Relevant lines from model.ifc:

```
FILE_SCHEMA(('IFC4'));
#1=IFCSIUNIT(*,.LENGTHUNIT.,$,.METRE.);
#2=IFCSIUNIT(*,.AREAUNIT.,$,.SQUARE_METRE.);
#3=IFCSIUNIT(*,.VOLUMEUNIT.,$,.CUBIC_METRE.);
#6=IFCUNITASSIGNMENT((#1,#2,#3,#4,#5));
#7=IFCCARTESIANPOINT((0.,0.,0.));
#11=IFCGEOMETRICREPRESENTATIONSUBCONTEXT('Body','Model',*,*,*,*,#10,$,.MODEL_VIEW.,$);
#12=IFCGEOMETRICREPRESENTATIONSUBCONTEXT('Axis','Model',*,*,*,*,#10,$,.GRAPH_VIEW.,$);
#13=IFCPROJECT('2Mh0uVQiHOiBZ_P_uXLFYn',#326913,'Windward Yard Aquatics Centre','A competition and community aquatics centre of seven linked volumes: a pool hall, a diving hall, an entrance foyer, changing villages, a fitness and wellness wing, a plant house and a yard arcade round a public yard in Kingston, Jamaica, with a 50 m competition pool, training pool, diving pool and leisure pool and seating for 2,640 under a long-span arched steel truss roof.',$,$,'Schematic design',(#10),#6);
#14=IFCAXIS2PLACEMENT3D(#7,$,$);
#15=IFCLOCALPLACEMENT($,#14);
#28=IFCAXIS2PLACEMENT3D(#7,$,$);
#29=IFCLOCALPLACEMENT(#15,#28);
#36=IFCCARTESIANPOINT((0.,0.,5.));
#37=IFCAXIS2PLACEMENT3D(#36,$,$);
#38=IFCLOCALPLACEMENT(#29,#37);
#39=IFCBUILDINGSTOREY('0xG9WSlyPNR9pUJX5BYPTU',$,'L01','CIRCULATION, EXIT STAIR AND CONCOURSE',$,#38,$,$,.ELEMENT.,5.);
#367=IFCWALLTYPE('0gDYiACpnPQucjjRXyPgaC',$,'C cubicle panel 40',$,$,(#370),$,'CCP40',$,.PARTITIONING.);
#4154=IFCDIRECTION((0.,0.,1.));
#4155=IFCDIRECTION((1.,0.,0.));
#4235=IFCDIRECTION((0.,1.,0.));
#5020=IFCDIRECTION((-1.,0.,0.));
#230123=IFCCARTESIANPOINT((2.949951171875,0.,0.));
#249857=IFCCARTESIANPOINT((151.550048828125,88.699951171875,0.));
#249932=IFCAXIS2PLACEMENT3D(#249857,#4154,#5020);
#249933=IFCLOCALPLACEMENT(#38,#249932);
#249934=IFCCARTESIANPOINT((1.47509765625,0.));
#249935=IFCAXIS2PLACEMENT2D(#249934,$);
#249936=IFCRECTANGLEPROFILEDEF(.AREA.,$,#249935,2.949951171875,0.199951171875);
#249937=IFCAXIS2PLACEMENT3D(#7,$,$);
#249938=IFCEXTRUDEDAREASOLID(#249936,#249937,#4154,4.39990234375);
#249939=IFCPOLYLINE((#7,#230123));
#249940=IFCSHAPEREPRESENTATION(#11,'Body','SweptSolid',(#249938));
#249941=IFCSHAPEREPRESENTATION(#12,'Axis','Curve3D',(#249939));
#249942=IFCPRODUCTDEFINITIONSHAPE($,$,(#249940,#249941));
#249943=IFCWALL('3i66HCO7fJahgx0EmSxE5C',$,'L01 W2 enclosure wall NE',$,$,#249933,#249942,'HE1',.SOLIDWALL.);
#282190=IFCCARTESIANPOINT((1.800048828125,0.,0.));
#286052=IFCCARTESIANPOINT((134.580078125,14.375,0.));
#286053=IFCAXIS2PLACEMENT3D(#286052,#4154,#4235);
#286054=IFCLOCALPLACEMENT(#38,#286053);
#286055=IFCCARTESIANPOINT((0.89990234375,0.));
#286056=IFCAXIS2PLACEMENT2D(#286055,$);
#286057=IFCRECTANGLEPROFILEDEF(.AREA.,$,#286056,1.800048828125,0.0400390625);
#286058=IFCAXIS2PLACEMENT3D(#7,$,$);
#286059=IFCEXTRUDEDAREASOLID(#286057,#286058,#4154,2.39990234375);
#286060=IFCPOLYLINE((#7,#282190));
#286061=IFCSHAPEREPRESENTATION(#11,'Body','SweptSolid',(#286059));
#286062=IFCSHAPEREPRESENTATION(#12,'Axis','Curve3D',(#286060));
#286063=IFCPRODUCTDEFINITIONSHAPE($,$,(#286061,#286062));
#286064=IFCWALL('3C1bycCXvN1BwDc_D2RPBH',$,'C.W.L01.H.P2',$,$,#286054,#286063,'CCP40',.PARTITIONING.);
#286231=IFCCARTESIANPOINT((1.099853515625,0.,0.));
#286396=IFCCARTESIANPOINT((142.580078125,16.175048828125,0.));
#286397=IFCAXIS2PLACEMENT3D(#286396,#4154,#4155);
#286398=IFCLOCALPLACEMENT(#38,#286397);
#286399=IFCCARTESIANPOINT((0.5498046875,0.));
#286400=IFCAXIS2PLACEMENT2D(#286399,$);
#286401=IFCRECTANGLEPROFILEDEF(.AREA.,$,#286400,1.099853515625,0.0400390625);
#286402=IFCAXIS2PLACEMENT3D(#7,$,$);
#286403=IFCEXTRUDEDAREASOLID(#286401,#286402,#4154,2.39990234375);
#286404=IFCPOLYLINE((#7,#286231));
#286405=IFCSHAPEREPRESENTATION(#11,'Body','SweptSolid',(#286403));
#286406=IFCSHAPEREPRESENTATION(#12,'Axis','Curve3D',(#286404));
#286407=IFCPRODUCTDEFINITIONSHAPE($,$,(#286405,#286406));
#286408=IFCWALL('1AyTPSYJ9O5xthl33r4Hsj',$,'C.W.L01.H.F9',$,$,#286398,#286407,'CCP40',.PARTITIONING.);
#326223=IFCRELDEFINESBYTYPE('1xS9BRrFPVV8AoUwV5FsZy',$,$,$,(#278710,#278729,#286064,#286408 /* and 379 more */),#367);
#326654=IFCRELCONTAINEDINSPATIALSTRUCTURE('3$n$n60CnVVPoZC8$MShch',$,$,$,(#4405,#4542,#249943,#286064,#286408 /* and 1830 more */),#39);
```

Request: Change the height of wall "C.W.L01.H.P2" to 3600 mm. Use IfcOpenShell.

```python
import ifcopenshell
import ifcopenshell.geom
import ifcopenshell.util.representation
import ifcopenshell.util.shape
import ifcopenshell.util.unit

model = ifcopenshell.open("model.ifc")
unit_scale = ifcopenshell.util.unit.calculate_unit_scale(model)
settings = ifcopenshell.geom.settings()


def volume(element):
    """Net volume in cubic metres, openings subtracted."""
    shape = ifcopenshell.geom.create_shape(settings, element)
    return ifcopenshell.util.shape.get_volume(shape.geometry)


wall = model.by_guid("3C1bycCXvN1BwDc_D2RPBH")
before = volume(wall)

body = ifcopenshell.util.representation.get_representation(wall, "Model", "Body")
solid = body.Items[0]
old_height = solid.Depth
solid.Depth = 3.6 / unit_scale
after = volume(wall)

print(f"height {old_height:g} -> {solid.Depth:g}, volume {before:.3f} -> {after:.3f} m3")

model.write("model_edited.ifc")
```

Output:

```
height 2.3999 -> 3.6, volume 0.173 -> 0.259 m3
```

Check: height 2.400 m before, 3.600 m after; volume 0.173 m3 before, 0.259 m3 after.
